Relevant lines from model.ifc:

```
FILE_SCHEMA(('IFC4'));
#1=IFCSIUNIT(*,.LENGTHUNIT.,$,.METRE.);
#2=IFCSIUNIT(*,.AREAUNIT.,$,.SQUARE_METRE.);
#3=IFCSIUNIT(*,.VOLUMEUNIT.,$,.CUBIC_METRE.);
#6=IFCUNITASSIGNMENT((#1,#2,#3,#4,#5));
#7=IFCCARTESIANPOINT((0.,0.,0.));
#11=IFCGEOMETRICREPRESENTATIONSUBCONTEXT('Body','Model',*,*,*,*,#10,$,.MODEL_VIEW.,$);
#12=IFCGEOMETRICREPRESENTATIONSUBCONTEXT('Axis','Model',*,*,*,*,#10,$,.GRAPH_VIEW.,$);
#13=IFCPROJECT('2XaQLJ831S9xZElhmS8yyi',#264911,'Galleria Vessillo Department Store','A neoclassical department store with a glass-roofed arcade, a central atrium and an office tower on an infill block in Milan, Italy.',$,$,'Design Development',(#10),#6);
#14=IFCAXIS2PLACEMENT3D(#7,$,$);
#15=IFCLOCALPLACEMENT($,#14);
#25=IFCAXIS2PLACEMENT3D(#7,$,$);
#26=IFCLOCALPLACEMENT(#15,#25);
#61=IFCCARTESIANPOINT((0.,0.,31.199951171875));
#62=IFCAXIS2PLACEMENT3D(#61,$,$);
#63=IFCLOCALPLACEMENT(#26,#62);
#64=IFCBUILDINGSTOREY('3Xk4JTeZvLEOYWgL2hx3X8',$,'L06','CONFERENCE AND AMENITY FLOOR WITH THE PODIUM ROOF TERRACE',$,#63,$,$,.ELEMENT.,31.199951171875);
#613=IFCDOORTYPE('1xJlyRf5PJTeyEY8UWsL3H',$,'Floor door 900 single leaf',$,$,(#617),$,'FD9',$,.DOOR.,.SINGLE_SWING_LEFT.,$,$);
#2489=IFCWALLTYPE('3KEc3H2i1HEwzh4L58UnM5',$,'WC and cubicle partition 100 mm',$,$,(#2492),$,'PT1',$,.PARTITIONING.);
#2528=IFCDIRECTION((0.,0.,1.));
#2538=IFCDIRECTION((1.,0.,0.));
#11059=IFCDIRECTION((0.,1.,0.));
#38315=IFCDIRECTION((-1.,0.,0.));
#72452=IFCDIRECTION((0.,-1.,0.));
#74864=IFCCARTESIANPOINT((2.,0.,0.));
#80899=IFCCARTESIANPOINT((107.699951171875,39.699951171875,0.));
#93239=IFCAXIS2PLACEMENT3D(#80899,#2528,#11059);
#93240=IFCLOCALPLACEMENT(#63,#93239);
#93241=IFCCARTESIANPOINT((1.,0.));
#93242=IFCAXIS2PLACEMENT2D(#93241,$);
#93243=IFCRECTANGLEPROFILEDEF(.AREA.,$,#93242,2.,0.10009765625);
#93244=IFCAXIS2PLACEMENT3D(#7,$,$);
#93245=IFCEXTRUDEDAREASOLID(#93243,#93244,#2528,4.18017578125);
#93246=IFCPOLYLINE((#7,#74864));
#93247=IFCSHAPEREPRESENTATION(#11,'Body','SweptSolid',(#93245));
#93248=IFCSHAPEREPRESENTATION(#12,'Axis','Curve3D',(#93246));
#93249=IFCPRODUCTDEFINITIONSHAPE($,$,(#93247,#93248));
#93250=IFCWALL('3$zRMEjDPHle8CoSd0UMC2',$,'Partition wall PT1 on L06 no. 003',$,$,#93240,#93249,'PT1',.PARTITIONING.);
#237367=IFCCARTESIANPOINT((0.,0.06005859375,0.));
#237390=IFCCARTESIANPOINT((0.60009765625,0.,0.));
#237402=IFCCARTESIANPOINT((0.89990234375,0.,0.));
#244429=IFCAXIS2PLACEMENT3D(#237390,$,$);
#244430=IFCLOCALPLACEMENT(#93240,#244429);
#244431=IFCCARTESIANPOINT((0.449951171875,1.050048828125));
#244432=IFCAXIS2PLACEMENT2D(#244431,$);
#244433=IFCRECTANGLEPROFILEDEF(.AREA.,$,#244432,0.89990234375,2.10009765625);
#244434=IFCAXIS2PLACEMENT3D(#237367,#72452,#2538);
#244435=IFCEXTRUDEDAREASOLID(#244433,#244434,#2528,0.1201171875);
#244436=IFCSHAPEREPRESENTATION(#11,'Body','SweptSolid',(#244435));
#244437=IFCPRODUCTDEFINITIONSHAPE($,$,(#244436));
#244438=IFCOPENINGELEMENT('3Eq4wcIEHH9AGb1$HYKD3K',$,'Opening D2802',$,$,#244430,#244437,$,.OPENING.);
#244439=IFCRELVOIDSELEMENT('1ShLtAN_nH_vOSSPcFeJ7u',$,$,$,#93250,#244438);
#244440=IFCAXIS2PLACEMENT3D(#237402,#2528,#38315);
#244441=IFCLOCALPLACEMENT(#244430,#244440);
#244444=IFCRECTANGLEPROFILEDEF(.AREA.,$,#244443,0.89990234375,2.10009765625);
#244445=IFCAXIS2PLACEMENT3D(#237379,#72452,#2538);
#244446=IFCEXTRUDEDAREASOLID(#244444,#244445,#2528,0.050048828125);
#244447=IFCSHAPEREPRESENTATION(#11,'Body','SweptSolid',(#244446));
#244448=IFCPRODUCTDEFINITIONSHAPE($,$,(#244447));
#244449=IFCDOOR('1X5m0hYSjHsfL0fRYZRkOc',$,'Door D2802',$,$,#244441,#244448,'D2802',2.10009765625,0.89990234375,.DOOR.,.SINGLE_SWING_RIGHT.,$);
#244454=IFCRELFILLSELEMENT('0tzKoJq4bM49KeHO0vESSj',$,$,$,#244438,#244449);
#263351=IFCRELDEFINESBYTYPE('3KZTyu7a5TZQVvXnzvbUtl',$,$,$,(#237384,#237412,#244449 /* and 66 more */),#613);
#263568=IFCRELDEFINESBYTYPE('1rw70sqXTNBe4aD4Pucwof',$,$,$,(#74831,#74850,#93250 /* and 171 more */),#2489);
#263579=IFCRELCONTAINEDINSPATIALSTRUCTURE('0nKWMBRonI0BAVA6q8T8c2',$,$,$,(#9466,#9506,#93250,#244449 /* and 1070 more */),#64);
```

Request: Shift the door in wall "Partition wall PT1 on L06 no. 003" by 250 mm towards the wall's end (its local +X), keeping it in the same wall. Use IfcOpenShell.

```python
import ifcopenshell
import ifcopenshell.api.geometry
import ifcopenshell.util.placement
import ifcopenshell.util.unit

model = ifcopenshell.open("model.ifc")
unit_scale = ifcopenshell.util.unit.calculate_unit_scale(model)

door = model.by_guid("1X5m0hYSjHsfL0fRYZRkOc")
opening = door.FillsVoids[0].RelatingOpeningElement
wall = opening.VoidsElements[0].RelatingBuildingElement

wall_matrix = ifcopenshell.util.placement.get_local_placement(wall.ObjectPlacement)
shift = wall_matrix[:3, 0] * 0.25 / unit_scale
before = ifcopenshell.util.placement.get_local_placement(door.ObjectPlacement)[:3, 3].copy()

# The door is placed relative to its opening, so it follows when the opening moves.
matrix = ifcopenshell.util.placement.get_local_placement(opening.ObjectPlacement)
matrix[:3, 3] += shift
ifcopenshell.api.geometry.edit_object_placement(
    model, product=opening, matrix=matrix, is_si=False, should_transform_children=True
)

after = ifcopenshell.util.placement.get_local_placement(door.ObjectPlacement)[:3, 3]
print("door moved by", (after - before).round(3) + 0.0)

model.write("model_updated.ifc")
```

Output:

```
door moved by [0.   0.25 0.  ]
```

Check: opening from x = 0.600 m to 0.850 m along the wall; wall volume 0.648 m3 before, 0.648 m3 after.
